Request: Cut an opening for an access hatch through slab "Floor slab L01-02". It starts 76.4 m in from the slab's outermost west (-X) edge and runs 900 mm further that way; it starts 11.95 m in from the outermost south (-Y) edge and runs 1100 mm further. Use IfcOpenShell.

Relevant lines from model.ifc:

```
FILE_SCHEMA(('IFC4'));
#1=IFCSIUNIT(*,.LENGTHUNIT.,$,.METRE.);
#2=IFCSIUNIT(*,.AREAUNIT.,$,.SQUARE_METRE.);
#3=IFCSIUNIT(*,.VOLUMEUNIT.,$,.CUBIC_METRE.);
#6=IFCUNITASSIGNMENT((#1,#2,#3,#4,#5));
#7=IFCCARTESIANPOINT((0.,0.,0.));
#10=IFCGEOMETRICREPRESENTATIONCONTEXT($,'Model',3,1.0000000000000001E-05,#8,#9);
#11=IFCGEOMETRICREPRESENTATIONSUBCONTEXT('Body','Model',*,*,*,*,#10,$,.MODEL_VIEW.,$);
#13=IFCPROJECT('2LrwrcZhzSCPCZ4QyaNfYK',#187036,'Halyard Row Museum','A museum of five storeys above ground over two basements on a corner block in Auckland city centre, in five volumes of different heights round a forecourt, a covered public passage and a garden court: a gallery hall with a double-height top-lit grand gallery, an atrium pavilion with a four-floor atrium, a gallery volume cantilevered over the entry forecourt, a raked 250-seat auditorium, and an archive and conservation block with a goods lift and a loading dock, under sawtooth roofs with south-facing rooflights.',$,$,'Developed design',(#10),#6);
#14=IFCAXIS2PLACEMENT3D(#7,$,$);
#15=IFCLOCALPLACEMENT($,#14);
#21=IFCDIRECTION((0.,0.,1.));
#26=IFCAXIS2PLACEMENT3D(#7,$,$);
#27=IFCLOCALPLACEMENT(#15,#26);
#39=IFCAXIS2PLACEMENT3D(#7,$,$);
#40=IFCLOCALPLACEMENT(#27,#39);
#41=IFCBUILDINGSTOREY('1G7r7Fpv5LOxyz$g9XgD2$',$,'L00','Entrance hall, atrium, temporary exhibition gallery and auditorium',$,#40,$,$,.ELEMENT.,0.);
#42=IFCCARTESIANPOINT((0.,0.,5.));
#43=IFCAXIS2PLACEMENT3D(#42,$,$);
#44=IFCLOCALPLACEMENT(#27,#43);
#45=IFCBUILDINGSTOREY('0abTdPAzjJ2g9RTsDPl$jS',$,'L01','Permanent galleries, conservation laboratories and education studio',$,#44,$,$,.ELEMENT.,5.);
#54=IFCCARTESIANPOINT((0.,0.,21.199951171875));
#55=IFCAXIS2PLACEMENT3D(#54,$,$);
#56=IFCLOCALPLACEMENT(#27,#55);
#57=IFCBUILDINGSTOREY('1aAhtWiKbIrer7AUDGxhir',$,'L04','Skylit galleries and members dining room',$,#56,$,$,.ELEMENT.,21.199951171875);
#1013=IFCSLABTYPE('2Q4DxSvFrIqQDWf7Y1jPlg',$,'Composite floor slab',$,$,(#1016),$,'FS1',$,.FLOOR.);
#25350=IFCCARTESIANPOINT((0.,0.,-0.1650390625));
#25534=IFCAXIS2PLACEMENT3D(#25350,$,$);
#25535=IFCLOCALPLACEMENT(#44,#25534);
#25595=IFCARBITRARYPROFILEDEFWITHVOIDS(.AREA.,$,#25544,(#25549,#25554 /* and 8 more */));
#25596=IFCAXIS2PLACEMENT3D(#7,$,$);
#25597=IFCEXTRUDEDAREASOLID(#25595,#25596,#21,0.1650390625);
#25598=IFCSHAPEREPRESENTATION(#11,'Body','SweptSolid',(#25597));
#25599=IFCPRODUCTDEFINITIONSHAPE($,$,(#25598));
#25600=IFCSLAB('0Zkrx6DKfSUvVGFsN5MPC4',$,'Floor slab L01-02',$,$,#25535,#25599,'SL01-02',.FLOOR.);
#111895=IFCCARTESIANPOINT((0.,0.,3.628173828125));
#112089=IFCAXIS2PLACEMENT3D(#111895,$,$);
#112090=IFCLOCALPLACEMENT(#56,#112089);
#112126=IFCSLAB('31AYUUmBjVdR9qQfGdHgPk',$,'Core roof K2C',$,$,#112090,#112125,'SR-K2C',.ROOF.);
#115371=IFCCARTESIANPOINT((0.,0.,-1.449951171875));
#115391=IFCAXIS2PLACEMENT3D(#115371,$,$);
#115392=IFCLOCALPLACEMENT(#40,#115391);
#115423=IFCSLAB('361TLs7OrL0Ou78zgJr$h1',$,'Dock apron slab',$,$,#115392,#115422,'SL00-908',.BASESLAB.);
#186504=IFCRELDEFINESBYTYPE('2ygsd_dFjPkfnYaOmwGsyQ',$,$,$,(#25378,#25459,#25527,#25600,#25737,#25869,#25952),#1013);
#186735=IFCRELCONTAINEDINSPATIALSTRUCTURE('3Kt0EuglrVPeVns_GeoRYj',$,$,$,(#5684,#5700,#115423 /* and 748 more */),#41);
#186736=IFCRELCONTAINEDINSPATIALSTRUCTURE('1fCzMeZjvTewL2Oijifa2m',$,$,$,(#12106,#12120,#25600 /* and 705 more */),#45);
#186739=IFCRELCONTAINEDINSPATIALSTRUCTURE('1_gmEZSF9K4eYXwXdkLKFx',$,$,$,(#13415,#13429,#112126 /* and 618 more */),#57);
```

```python
import numpy as np
import ifcopenshell
import ifcopenshell.api.feature
import ifcopenshell.api.geometry
import ifcopenshell.api.root
import ifcopenshell.geom
import ifcopenshell.util.placement
import ifcopenshell.util.representation
import ifcopenshell.util.shape
import ifcopenshell.util.unit

model = ifcopenshell.open("model.ifc")
unit_scale = ifcopenshell.util.unit.calculate_unit_scale(model)
settings = ifcopenshell.geom.settings()


def volume(element):
    """Net volume in cubic metres, openings subtracted."""
    shape = ifcopenshell.geom.create_shape(settings, element)
    return ifcopenshell.util.shape.get_volume(shape.geometry)


slab = model.by_guid("0Zkrx6DKfSUvVGFsN5MPC4")
before = volume(slab)

# Extent in the slab's own axes, in metres. The edges named are its -X and -Y sides.
slab_shape = ifcopenshell.geom.create_shape(settings, slab)
vertices = ifcopenshell.util.shape.get_vertices(slab_shape.geometry)
x_min, y_min, bottom = vertices.min(axis=0)
top = vertices[:, 2].max()

opening = ifcopenshell.api.root.create_entity(model, ifc_class="IfcOpeningElement", name="Access hatch opening", predefined_type="OPENING")
context = ifcopenshell.util.representation.get_context(model, "Model", "Body", "MODEL_VIEW")
width, depth = 0.9, 1.1
outline = [(0.0, 0.0), (width, 0.0), (width, depth), (0.0, depth), (0.0, 0.0)]
# Overshoot both faces by 50 mm so the cut is clean.
shape = ifcopenshell.api.geometry.add_slab_representation(
    model, context=context, depth=top - bottom + 0.1, polyline=outline
)
ifcopenshell.api.geometry.assign_representation(model, product=opening, representation=shape)

matrix = ifcopenshell.util.placement.get_local_placement(slab.ObjectPlacement)
matrix[:, 3] = matrix @ np.append(np.array([x_min + 76.4, y_min + 11.95, bottom - 0.05]) / unit_scale, 1.0)
ifcopenshell.api.geometry.edit_object_placement(model, product=opening, matrix=matrix, is_si=False)
ifcopenshell.api.feature.add_feature(model, feature=opening, element=slab)

after = volume(slab)

print(f"slab volume {before:.3f} -> {after:.3f} m3")

model.write("model_rev.ifc")
```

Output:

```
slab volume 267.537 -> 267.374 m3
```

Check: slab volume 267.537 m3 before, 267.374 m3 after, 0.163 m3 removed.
